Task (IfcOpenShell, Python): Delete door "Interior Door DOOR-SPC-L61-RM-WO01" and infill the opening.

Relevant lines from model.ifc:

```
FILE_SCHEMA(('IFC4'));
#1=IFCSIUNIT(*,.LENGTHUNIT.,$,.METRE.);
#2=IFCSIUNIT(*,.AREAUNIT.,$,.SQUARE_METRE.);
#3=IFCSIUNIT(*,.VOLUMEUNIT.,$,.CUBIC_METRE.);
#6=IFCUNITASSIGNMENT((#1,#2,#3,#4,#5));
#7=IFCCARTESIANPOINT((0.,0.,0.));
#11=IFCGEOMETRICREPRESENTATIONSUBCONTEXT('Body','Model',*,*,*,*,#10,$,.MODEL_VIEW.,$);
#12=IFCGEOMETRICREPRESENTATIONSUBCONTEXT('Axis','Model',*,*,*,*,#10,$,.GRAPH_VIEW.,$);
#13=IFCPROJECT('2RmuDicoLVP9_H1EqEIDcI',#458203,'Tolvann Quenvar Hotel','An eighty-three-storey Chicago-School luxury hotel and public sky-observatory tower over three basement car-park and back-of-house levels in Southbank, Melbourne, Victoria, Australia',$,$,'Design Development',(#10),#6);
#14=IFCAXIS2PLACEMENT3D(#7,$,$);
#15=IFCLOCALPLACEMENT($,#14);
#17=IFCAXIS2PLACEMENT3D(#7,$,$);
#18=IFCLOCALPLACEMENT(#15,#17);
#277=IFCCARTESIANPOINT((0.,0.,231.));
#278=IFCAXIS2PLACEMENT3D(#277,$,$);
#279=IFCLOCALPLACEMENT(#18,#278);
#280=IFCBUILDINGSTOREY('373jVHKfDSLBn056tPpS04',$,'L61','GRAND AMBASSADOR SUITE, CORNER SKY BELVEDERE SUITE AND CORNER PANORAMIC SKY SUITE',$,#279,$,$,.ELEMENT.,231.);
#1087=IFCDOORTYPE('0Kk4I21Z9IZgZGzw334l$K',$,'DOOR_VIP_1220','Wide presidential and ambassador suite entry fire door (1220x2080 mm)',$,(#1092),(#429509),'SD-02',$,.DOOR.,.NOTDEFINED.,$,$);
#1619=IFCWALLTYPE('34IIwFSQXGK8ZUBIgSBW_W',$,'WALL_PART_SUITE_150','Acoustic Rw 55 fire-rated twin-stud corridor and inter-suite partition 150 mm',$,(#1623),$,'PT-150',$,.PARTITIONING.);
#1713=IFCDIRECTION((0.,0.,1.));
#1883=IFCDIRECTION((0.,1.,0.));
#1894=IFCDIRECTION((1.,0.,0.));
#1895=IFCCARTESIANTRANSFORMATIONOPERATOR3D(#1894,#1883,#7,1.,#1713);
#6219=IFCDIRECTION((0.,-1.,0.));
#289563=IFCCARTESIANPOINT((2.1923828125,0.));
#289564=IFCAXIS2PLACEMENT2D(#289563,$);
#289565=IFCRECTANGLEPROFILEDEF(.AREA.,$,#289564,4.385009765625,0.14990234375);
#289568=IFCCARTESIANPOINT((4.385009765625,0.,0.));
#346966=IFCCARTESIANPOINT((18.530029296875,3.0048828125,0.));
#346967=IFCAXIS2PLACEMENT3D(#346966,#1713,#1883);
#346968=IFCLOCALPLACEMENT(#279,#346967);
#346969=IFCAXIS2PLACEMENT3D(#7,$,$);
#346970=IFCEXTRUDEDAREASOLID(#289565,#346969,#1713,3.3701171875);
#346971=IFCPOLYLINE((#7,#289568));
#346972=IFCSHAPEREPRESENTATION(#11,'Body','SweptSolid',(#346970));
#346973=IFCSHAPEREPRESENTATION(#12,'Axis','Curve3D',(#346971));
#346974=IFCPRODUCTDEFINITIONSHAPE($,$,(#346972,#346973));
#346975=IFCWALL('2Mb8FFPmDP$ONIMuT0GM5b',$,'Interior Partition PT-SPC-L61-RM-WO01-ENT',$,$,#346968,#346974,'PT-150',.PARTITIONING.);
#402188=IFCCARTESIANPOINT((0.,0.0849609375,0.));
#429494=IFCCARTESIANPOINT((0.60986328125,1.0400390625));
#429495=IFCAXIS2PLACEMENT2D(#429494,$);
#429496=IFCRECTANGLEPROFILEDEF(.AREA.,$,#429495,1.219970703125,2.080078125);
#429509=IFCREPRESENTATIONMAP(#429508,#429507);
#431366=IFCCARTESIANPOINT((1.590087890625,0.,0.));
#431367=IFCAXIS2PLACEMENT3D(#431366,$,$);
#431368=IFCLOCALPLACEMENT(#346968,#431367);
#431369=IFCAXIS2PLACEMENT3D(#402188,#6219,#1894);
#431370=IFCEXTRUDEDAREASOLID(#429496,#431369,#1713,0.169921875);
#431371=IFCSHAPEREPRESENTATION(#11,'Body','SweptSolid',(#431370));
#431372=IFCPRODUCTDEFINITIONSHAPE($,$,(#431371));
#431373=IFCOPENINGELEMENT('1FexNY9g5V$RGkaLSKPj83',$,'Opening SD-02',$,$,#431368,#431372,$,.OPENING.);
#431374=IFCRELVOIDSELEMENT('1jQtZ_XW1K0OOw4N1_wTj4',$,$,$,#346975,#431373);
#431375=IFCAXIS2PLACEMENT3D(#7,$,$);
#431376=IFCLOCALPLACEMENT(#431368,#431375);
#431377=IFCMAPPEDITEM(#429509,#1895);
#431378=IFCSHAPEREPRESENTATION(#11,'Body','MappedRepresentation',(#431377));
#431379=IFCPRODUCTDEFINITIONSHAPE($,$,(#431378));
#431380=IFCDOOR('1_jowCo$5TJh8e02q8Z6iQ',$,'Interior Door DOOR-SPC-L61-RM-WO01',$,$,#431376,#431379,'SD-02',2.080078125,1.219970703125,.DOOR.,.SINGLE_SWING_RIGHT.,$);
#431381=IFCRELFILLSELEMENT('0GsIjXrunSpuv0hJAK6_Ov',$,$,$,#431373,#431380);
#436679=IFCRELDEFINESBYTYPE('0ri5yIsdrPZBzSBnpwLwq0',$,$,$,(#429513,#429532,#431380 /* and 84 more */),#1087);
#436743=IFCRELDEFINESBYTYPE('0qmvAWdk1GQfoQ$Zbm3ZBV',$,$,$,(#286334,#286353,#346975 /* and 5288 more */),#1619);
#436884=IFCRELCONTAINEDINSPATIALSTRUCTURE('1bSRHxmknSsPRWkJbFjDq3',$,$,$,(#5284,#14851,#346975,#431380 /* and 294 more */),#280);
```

```python
import ifcopenshell
import ifcopenshell.api.feature
import ifcopenshell.api.root
import ifcopenshell.geom
import ifcopenshell.util.shape

model = ifcopenshell.open("model.ifc")
settings = ifcopenshell.geom.settings()


def volume(element):
    """Net volume in cubic metres, openings subtracted."""
    shape = ifcopenshell.geom.create_shape(settings, element)
    return ifcopenshell.util.shape.get_volume(shape.geometry)


door = model.by_id(431380)
opening = door.FillsVoids[0].RelatingOpeningElement
wall = opening.VoidsElements[0].RelatingBuildingElement
before = volume(wall)

ifcopenshell.api.root.remove_product(model, product=door)
ifcopenshell.api.feature.remove_feature(model, feature=opening)

after = volume(wall)

print(f"wall volume {before:.3f} -> {after:.3f} m3")

model.write("model-out.ifc")
```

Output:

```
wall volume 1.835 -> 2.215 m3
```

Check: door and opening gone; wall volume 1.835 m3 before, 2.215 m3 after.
